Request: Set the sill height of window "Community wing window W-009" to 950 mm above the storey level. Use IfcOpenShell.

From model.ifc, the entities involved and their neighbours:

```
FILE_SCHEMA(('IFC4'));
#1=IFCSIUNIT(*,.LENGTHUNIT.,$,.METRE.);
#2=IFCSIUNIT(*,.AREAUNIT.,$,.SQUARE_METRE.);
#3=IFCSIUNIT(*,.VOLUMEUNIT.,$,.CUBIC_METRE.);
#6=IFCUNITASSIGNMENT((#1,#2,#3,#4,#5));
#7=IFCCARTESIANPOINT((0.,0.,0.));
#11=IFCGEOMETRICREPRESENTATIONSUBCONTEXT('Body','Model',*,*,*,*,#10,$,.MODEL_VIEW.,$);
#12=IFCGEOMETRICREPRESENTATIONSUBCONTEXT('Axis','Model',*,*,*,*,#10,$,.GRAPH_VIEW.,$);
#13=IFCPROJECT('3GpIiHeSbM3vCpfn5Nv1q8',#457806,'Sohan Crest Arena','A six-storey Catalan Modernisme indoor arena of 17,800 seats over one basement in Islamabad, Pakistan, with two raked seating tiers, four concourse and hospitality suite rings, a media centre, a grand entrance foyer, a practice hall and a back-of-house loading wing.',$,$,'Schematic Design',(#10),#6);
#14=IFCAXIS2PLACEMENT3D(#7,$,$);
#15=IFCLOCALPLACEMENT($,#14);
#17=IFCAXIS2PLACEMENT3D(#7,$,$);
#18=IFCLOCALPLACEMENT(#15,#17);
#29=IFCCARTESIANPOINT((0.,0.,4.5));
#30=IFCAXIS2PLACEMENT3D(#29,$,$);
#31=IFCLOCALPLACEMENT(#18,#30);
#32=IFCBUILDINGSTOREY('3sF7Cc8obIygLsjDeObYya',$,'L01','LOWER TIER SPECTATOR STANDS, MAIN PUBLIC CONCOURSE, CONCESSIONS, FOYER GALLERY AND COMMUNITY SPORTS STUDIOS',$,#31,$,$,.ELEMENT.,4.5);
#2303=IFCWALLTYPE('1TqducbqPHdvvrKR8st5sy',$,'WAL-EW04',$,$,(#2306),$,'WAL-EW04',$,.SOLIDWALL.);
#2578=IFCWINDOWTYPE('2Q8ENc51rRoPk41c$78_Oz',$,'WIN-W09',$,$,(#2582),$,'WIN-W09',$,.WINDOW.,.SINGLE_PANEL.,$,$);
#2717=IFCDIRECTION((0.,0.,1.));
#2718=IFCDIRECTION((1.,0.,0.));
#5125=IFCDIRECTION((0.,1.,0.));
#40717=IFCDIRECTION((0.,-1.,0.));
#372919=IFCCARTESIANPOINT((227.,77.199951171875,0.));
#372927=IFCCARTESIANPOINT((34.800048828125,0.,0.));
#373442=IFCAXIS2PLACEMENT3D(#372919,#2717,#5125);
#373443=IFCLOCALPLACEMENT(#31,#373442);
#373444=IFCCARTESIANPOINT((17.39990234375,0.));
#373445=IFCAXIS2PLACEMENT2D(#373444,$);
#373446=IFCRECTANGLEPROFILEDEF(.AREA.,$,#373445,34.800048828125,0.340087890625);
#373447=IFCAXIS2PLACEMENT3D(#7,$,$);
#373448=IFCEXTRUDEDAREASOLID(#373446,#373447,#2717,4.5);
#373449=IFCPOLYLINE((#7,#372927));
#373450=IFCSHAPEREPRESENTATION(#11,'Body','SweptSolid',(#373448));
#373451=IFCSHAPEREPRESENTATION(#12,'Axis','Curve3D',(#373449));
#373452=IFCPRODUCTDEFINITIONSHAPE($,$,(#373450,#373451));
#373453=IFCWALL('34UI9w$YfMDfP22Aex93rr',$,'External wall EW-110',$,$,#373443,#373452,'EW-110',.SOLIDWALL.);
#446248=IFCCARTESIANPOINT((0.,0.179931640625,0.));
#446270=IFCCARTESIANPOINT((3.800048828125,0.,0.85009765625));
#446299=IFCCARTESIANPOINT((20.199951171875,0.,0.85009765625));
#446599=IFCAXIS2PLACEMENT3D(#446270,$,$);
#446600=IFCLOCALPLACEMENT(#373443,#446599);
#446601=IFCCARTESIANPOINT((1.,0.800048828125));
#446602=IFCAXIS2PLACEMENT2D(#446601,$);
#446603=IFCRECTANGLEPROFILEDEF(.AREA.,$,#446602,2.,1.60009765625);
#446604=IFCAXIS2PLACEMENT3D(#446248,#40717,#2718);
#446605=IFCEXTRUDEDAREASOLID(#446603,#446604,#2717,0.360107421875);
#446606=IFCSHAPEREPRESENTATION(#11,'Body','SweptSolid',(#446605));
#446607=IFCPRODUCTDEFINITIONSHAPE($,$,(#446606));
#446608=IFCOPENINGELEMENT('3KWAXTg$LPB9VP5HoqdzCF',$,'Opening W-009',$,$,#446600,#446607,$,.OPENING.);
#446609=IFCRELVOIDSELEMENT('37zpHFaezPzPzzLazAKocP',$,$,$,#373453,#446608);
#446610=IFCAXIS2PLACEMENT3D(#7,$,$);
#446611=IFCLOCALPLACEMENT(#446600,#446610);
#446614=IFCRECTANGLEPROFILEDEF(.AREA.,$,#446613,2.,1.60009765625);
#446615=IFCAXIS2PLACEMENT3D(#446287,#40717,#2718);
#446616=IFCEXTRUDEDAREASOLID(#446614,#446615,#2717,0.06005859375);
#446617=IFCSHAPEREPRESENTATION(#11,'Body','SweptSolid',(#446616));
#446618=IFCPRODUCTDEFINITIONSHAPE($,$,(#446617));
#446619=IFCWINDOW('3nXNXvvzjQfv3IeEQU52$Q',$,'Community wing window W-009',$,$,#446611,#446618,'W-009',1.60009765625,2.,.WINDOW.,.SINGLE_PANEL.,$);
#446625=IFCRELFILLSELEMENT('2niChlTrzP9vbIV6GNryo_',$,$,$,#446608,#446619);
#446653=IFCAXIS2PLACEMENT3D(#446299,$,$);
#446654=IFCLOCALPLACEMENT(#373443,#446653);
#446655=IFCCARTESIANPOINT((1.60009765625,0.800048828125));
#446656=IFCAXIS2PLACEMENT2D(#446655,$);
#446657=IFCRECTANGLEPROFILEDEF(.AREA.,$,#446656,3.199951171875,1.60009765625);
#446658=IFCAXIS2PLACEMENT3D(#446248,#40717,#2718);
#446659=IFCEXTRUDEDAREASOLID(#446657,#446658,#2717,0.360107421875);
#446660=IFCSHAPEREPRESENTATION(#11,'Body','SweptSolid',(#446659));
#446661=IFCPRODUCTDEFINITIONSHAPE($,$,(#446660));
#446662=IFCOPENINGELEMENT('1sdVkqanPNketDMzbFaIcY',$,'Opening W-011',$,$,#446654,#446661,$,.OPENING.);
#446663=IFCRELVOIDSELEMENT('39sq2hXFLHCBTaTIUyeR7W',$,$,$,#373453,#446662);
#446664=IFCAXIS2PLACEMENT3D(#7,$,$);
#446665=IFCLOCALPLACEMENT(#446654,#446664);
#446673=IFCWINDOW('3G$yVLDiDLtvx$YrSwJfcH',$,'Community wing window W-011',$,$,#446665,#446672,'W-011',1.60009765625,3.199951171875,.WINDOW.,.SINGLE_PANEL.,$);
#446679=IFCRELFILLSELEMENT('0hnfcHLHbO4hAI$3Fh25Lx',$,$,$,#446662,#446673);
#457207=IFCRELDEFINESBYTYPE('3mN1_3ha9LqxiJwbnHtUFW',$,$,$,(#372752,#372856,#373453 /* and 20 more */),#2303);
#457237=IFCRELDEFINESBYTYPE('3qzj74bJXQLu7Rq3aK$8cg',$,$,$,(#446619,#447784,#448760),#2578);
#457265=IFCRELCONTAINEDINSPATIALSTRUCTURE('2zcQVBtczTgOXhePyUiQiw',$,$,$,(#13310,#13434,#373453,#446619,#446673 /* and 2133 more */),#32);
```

```python
import numpy as np
import ifcopenshell
import ifcopenshell.api.geometry
import ifcopenshell.geom
import ifcopenshell.util.element
import ifcopenshell.util.placement
import ifcopenshell.util.shape
import ifcopenshell.util.unit

model = ifcopenshell.open("model.ifc")
unit_scale = ifcopenshell.util.unit.calculate_unit_scale(model)

window = model.by_id(446619)
opening = window.FillsVoids[0].RelatingOpeningElement
storey = ifcopenshell.util.element.get_container(window, ifc_class="IfcBuildingStorey")
level = ifcopenshell.util.placement.get_local_placement(storey.ObjectPlacement)[2, 3]

# The opening's origin need not be at the sill, so measure its lowest point.
shape = ifcopenshell.geom.create_shape(ifcopenshell.geom.settings(), opening)
bottom = ifcopenshell.util.shape.get_shape_bottom_elevation(shape, shape.geometry) / unit_scale
dz = level + 0.95 / unit_scale - bottom

shift = np.array([0.0, 0.0, dz])
# The window is placed relative to its opening, so it follows when the opening moves.
matrix = ifcopenshell.util.placement.get_local_placement(opening.ObjectPlacement)
matrix[:3, 3] += shift
ifcopenshell.api.geometry.edit_object_placement(
    model, product=opening, matrix=matrix, is_si=False, should_transform_children=True
)

print(f"moved by {dz * unit_scale:+.3f} m")

model.write("model_edited.ifc")
```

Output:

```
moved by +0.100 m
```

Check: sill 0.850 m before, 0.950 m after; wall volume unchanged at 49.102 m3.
